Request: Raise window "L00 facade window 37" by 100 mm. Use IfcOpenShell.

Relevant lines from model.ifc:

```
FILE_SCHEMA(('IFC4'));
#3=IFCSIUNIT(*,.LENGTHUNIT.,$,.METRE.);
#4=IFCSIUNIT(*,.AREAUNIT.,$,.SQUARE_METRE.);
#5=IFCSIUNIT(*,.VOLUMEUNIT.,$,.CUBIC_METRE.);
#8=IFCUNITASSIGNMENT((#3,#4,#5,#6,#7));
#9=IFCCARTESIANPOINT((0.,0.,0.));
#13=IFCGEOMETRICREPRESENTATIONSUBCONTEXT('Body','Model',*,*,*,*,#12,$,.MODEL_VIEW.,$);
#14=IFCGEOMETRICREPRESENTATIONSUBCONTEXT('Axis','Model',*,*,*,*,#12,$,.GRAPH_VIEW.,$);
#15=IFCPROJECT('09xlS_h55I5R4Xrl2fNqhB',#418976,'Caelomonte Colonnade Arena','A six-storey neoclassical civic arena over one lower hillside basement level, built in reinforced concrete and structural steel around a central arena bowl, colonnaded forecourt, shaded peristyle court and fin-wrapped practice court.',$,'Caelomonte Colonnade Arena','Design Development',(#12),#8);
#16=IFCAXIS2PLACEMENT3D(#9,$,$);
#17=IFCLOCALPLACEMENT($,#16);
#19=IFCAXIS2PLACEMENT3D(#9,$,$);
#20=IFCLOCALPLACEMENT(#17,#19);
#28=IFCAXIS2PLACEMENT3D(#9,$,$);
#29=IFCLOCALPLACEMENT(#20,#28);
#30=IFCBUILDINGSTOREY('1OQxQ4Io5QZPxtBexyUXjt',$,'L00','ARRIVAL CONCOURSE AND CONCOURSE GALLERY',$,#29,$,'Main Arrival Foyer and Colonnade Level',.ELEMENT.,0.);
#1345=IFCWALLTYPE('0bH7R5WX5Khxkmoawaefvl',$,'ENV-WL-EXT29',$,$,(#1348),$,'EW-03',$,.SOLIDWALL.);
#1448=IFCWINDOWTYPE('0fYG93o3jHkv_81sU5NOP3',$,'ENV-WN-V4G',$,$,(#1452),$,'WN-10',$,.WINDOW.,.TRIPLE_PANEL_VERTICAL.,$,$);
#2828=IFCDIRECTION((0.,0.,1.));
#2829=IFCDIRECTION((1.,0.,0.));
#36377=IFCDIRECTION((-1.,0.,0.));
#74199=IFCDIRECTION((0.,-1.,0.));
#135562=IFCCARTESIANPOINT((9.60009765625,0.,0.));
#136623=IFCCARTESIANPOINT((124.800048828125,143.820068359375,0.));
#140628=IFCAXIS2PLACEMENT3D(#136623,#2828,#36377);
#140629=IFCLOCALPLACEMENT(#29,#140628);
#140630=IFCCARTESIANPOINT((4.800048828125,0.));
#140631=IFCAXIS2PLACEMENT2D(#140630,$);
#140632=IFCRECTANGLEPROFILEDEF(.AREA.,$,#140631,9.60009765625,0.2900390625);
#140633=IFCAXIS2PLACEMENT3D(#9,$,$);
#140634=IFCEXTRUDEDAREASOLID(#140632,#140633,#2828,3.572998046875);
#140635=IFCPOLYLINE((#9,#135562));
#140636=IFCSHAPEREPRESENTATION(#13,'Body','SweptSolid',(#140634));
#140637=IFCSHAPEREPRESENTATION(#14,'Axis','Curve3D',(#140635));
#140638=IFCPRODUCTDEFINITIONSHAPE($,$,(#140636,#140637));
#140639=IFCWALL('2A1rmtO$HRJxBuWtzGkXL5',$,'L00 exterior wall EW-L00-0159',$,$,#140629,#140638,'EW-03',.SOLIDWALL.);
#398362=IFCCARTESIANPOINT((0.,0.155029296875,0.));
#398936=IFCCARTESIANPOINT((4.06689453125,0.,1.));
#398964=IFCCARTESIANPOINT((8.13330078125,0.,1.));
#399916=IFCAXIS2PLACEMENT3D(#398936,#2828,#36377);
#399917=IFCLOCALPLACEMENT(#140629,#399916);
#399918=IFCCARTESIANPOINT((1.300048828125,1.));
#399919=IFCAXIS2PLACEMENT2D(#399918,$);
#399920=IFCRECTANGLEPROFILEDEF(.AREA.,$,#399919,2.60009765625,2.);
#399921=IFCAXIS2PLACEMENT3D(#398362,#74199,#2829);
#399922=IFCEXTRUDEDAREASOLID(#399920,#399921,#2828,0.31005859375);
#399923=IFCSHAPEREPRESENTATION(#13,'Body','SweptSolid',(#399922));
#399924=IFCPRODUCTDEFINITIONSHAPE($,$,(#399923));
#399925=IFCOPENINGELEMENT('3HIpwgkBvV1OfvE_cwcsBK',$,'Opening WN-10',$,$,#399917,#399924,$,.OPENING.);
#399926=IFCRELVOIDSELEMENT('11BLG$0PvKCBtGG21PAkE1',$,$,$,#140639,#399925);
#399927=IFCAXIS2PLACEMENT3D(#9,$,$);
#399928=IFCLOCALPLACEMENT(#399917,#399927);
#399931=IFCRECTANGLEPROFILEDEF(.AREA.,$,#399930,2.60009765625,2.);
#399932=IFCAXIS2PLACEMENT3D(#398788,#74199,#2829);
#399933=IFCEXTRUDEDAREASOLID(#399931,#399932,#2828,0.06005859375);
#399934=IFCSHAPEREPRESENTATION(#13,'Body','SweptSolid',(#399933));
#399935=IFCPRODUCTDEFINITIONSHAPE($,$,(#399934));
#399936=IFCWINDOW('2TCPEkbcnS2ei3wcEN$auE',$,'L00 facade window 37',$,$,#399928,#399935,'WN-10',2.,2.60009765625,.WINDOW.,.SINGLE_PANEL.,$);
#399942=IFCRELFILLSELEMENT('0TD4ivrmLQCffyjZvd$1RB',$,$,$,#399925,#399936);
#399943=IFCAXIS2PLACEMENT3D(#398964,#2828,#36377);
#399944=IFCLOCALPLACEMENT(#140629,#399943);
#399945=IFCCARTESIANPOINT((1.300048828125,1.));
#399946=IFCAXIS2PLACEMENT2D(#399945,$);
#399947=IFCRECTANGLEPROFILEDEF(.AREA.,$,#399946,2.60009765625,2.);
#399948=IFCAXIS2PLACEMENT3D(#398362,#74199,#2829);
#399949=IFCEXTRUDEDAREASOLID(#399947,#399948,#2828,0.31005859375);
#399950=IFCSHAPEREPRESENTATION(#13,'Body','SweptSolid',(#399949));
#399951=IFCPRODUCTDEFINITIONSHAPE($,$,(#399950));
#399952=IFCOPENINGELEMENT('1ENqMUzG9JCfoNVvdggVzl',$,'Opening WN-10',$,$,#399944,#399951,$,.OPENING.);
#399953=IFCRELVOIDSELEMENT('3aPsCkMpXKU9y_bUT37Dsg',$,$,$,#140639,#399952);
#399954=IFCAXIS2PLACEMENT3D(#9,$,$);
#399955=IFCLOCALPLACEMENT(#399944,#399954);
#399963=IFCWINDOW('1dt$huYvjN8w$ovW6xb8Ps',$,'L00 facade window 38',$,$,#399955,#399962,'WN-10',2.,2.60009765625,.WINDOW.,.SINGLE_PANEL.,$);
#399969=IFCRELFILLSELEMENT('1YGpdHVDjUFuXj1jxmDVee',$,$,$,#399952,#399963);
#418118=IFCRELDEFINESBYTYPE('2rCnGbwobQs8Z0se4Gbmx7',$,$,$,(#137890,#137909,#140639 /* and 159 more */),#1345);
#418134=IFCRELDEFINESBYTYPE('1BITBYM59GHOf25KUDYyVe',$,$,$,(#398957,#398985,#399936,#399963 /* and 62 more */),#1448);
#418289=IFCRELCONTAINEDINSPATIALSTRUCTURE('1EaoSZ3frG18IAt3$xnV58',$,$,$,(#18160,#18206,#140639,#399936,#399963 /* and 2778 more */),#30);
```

```python
import numpy as np
import ifcopenshell
import ifcopenshell.api.geometry
import ifcopenshell.util.placement
import ifcopenshell.util.unit

model = ifcopenshell.open("model.ifc")
unit_scale = ifcopenshell.util.unit.calculate_unit_scale(model)

window = model.by_id(399936)
opening = window.FillsVoids[0].RelatingOpeningElement
dz = 0.1

shift = np.array([0.0, 0.0, dz])
# The window is placed relative to its opening, so it follows when the opening moves.
matrix = ifcopenshell.util.placement.get_local_placement(opening.ObjectPlacement)
matrix[:3, 3] += shift
ifcopenshell.api.geometry.edit_object_placement(
    model, product=opening, matrix=matrix, is_si=False, should_transform_children=True
)

print(f"moved by {dz * unit_scale:+.3f} m")

model.write("model_updated.ifc")
```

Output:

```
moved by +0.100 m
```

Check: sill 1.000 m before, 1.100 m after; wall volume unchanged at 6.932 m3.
